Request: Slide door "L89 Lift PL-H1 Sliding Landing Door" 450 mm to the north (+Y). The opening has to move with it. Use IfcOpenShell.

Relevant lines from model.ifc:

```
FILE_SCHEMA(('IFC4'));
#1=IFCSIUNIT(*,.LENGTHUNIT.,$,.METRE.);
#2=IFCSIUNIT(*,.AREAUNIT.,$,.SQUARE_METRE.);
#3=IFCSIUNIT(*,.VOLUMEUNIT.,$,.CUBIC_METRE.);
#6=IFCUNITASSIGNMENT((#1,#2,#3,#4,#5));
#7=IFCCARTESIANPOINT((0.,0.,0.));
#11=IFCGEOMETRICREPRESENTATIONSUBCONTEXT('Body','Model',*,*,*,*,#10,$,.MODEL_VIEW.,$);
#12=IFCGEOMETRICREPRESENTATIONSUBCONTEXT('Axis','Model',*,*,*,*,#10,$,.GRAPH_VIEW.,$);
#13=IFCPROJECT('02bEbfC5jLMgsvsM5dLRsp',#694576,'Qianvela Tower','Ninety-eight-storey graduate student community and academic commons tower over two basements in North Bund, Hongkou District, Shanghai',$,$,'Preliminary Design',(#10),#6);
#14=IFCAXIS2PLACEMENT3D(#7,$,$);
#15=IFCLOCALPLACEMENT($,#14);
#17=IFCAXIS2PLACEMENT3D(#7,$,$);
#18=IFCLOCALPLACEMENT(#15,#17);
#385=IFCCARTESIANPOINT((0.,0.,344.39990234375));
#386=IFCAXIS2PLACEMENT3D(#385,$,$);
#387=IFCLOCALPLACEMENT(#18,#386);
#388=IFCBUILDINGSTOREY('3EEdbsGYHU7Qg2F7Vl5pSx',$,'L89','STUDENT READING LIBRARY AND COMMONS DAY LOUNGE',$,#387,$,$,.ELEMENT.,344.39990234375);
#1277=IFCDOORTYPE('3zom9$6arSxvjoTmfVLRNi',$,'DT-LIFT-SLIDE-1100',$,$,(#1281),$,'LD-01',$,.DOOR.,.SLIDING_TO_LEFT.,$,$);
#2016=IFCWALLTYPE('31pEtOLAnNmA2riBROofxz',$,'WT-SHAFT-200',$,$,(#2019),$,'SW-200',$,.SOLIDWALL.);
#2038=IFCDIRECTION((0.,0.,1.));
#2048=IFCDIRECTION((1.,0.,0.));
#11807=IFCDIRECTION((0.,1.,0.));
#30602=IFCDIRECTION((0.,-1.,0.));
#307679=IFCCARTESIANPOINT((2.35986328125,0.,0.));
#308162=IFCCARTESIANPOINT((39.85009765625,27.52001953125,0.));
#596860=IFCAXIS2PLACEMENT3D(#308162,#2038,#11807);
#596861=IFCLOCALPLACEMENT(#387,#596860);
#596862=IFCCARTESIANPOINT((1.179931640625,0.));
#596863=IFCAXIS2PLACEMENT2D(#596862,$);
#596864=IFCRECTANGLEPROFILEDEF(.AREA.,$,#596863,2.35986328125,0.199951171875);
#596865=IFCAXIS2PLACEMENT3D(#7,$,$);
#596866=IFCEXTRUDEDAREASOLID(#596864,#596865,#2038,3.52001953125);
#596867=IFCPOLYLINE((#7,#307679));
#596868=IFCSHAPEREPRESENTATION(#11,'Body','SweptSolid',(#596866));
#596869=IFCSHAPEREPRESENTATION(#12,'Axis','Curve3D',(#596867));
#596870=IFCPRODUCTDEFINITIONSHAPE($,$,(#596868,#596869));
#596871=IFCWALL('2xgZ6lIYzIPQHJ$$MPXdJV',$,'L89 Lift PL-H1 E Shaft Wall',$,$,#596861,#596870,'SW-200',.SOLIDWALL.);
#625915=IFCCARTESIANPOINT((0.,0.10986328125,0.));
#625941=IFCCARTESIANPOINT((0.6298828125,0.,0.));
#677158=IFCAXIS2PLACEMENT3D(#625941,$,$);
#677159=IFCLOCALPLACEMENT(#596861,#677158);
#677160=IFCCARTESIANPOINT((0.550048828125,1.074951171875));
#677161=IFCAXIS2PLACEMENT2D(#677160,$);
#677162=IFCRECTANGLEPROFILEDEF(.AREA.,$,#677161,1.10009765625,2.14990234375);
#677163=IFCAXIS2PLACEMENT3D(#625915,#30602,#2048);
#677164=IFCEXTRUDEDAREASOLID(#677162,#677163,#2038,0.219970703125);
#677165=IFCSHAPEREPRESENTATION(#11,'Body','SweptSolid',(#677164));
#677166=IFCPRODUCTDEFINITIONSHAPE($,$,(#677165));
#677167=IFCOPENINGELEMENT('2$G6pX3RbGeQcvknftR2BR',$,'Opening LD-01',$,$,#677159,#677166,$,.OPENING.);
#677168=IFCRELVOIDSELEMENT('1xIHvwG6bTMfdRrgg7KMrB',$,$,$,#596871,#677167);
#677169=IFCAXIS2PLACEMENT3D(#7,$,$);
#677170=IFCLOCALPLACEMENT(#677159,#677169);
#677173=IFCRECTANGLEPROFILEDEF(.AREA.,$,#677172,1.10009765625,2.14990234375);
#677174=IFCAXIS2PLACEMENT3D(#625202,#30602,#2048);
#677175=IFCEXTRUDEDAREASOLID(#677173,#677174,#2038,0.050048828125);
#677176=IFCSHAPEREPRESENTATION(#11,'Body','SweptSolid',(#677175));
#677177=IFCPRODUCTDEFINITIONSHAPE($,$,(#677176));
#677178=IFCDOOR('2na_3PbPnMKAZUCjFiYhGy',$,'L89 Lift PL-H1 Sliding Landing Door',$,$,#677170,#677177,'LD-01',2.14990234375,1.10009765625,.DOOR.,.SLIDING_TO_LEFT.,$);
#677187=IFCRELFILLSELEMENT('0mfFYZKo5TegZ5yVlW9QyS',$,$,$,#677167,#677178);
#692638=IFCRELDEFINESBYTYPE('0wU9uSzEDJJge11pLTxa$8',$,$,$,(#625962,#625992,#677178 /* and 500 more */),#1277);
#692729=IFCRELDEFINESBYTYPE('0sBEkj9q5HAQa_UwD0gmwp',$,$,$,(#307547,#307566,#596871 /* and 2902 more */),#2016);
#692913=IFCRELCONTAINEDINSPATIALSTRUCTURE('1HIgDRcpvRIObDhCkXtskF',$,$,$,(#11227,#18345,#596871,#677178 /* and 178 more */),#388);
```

```python
import ifcopenshell
import ifcopenshell.api.geometry
import ifcopenshell.util.placement

model = ifcopenshell.open("model.ifc")

door = model.by_id(677178)
opening = door.FillsVoids[0].RelatingOpeningElement
wall = opening.VoidsElements[0].RelatingBuildingElement

wall_matrix = ifcopenshell.util.placement.get_local_placement(wall.ObjectPlacement)
shift = wall_matrix[:3, 0] * 0.45
before = ifcopenshell.util.placement.get_local_placement(door.ObjectPlacement)[:3, 3].copy()

# The door is placed relative to its opening, so it follows when the opening moves.
matrix = ifcopenshell.util.placement.get_local_placement(opening.ObjectPlacement)
matrix[:3, 3] += shift
ifcopenshell.api.geometry.edit_object_placement(
    model, product=opening, matrix=matrix, is_si=False, should_transform_children=True
)

after = ifcopenshell.util.placement.get_local_placement(door.ObjectPlacement)[:3, 3]
print("door moved by", (after - before).round(3) + 0.0)

model.write("model-out.ifc")
```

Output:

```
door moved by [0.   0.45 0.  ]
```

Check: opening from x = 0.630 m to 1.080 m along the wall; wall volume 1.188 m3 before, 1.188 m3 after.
